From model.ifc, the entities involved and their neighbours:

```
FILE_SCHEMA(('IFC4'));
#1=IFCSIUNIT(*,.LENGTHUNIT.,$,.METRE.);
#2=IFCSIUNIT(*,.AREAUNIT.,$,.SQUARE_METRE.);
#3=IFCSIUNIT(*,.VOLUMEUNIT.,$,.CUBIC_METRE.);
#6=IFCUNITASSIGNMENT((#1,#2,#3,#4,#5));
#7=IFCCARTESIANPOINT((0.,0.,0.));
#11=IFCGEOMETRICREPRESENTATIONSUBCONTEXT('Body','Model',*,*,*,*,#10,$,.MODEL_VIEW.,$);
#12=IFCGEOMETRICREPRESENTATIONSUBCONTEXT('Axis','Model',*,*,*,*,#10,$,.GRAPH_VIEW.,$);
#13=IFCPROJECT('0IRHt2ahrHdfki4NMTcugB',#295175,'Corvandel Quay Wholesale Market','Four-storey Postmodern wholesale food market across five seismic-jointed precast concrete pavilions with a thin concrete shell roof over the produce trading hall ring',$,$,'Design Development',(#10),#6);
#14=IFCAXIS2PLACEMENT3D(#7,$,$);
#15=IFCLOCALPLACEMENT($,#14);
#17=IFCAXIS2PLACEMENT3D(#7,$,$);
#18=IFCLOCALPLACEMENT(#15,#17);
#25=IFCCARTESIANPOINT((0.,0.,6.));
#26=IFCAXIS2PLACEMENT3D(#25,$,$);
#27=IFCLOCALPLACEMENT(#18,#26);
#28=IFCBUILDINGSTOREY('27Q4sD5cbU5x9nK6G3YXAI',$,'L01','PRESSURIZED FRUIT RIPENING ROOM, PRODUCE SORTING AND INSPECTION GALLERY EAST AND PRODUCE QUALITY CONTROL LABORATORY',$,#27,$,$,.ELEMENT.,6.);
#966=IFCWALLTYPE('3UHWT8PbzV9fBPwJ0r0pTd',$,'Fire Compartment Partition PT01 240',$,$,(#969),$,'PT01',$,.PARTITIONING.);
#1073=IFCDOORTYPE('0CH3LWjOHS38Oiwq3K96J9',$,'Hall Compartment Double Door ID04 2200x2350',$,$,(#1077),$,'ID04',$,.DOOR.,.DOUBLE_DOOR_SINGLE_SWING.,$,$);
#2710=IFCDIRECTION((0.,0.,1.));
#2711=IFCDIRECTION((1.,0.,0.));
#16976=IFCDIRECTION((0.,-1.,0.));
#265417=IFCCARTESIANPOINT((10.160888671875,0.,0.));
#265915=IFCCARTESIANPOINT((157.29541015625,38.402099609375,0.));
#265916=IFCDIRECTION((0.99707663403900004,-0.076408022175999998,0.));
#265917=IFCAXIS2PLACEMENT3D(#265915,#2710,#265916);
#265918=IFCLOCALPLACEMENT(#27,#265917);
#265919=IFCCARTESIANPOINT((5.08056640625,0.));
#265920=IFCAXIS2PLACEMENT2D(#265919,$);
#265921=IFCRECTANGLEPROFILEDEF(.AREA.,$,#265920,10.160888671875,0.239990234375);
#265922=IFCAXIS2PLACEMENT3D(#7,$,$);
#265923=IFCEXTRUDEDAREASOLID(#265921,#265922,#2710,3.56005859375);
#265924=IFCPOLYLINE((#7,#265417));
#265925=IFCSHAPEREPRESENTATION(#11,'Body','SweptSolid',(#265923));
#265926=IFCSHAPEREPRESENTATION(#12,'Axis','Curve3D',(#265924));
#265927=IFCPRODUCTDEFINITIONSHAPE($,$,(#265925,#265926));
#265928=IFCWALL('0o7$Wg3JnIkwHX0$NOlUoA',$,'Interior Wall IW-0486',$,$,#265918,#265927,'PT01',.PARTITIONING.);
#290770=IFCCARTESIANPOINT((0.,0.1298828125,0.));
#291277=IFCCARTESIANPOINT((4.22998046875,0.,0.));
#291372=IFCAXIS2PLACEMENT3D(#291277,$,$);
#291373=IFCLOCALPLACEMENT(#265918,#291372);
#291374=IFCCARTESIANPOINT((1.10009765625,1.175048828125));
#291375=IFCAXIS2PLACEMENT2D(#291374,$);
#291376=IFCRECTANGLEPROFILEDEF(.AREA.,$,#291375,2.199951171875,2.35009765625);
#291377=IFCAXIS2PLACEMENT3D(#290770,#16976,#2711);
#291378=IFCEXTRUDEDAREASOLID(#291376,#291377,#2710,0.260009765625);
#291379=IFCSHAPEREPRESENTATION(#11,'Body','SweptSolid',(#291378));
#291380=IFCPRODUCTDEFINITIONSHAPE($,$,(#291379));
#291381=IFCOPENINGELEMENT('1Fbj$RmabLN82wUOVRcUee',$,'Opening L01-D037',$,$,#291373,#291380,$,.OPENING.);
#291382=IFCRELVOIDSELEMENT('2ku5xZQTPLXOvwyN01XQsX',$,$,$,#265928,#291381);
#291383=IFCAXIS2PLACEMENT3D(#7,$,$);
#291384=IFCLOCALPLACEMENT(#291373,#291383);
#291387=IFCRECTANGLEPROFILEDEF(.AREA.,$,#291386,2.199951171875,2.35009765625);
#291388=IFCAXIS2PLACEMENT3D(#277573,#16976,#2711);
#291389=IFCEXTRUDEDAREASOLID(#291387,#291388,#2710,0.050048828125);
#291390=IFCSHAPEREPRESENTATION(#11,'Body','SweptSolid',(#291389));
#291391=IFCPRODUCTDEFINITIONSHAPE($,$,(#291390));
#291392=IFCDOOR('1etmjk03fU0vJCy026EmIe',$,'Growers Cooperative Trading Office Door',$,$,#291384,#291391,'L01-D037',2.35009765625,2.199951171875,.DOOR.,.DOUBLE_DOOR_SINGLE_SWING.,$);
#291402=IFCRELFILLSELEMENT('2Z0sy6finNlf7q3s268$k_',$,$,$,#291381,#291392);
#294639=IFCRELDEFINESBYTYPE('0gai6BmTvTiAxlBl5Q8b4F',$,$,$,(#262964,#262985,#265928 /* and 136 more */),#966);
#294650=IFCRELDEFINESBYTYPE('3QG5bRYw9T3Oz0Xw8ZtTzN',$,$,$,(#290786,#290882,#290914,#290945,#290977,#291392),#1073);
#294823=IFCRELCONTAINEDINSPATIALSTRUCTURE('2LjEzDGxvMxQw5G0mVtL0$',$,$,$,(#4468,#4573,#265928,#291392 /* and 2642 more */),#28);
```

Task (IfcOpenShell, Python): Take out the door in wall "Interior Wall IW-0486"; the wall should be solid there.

```python
import ifcopenshell
import ifcopenshell.api.feature
import ifcopenshell.api.root
import ifcopenshell.geom
import ifcopenshell.util.shape

model = ifcopenshell.open("model.ifc")
settings = ifcopenshell.geom.settings()


def volume(element):
    """Net volume in cubic metres, openings subtracted."""
    shape = ifcopenshell.geom.create_shape(settings, element)
    return ifcopenshell.util.shape.get_volume(shape.geometry)


door = model.by_guid("1etmjk03fU0vJCy026EmIe")
opening = door.FillsVoids[0].RelatingOpeningElement
wall = opening.VoidsElements[0].RelatingBuildingElement
before = volume(wall)

ifcopenshell.api.root.remove_product(model, product=door)
ifcopenshell.api.feature.remove_feature(model, feature=opening)

after = volume(wall)

print(f"wall volume {before:.3f} -> {after:.3f} m3")

model.write("model_rev.ifc")
```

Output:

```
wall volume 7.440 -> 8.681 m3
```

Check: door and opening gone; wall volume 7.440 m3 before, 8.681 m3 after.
